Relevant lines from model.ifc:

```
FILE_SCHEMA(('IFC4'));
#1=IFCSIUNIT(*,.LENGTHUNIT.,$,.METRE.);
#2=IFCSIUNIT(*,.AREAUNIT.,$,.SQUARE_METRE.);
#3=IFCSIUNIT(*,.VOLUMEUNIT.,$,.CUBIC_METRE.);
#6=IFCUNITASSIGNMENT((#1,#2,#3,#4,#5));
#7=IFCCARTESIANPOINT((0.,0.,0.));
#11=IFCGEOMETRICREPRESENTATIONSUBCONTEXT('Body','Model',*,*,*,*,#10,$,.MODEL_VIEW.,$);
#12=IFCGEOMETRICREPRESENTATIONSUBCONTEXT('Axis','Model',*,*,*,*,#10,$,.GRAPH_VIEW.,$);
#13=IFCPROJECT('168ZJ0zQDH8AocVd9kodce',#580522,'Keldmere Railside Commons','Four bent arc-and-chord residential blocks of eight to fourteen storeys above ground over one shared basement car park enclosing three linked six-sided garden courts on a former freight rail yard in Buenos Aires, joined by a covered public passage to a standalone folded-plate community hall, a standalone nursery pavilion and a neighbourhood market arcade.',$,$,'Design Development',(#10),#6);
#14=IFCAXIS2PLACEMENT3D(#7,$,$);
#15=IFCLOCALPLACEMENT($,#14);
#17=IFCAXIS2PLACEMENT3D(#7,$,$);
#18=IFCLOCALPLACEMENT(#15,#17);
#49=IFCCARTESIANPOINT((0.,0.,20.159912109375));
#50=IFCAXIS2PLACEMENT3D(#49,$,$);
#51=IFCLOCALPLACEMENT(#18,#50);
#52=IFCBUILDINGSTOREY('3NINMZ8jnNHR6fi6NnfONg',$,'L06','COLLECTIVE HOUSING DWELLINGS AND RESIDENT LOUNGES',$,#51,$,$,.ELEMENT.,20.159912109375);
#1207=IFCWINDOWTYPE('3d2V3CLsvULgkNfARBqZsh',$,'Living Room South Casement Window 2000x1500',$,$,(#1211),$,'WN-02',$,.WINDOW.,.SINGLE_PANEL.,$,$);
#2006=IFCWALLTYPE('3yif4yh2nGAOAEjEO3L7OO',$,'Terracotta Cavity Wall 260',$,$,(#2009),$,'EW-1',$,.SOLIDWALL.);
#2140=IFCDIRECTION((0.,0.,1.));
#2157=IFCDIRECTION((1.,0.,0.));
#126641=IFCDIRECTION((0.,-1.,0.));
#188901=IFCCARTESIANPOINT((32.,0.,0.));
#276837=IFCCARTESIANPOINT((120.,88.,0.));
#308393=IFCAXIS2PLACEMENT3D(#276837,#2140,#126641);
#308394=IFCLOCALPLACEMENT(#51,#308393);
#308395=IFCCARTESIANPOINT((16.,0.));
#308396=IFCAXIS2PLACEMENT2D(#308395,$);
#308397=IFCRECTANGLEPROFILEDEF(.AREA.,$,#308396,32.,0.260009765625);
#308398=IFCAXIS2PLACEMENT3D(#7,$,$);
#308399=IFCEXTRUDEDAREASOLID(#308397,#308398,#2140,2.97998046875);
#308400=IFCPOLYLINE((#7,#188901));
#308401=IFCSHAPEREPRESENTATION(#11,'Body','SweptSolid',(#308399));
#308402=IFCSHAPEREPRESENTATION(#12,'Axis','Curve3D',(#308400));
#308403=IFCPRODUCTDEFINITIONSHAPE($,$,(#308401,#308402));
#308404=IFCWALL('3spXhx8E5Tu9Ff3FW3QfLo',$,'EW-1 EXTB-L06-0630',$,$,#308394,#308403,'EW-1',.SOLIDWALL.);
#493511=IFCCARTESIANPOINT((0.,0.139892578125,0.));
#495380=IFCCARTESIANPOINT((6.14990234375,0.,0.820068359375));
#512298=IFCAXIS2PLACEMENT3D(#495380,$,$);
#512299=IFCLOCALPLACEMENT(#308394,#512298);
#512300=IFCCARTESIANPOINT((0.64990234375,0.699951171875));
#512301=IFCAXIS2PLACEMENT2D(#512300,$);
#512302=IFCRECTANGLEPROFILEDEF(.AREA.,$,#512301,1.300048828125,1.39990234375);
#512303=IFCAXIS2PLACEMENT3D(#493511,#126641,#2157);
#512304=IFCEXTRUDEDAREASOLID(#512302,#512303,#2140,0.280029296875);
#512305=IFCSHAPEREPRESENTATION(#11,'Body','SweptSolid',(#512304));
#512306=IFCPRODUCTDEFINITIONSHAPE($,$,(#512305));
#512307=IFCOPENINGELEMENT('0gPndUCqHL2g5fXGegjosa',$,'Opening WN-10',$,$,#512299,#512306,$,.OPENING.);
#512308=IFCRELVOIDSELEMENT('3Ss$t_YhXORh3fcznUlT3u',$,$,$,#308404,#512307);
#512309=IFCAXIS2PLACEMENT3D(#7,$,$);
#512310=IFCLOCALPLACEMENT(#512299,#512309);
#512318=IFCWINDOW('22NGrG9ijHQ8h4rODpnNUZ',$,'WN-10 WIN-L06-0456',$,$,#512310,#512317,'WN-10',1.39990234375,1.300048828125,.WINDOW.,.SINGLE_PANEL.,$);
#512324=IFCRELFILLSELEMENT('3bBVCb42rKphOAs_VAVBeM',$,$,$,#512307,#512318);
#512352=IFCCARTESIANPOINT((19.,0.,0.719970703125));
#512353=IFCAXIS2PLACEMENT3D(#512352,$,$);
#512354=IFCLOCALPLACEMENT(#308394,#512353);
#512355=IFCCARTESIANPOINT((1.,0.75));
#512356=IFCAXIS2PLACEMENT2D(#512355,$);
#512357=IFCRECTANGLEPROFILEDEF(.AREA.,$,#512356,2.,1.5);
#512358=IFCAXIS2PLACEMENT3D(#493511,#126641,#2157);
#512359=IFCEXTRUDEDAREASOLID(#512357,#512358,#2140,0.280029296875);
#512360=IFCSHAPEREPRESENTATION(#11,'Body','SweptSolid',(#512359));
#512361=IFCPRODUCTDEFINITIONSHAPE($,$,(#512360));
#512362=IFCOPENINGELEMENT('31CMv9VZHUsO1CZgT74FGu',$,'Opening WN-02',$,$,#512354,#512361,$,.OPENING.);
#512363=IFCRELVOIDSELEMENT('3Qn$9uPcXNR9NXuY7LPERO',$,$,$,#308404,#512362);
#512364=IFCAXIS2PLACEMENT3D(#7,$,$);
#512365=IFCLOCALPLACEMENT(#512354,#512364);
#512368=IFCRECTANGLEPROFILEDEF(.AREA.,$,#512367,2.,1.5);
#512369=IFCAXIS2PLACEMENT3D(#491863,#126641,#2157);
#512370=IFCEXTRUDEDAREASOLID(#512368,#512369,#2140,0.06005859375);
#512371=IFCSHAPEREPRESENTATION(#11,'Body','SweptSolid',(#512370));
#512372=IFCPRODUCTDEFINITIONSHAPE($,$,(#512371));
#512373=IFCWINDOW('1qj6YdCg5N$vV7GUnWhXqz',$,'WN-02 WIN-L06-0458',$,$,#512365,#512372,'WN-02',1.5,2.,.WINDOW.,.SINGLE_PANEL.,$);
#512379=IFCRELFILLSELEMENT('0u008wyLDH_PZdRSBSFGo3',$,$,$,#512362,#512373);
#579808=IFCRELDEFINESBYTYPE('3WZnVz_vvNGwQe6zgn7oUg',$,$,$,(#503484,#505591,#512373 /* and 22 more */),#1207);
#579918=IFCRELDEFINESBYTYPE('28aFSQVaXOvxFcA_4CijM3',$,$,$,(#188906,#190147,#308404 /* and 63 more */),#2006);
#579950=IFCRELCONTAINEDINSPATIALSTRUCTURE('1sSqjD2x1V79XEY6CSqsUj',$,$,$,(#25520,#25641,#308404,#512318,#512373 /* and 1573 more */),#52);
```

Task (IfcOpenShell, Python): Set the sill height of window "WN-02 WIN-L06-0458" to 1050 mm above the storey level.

```python
import numpy as np
import ifcopenshell
import ifcopenshell.api.geometry
import ifcopenshell.geom
import ifcopenshell.util.element
import ifcopenshell.util.placement
import ifcopenshell.util.shape
import ifcopenshell.util.unit

model = ifcopenshell.open("model.ifc")
unit_scale = ifcopenshell.util.unit.calculate_unit_scale(model)

window = model.by_guid("1qj6YdCg5N$vV7GUnWhXqz")
opening = window.FillsVoids[0].RelatingOpeningElement
storey = ifcopenshell.util.element.get_container(window, ifc_class="IfcBuildingStorey")
level = ifcopenshell.util.placement.get_local_placement(storey.ObjectPlacement)[2, 3]

# The opening's origin need not be at the sill, so measure its lowest point.
shape = ifcopenshell.geom.create_shape(ifcopenshell.geom.settings(), opening)
bottom = ifcopenshell.util.shape.get_shape_bottom_elevation(shape, shape.geometry) / unit_scale
dz = level + 1.05 - bottom

shift = np.array([0.0, 0.0, dz])
# The window is placed relative to its opening, so it follows when the opening moves.
matrix = ifcopenshell.util.placement.get_local_placement(opening.ObjectPlacement)
matrix[:3, 3] += shift
ifcopenshell.api.geometry.edit_object_placement(
    model, product=opening, matrix=matrix, is_si=False, should_transform_children=True
)

print(f"moved by {dz * unit_scale:+.3f} m")

model.write("model_rev.ifc")
```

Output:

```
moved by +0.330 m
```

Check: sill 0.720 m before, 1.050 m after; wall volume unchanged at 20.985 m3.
